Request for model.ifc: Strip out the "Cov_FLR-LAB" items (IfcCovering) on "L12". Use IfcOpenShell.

First a look at what the model holds.

```python
import ifcopenshell
import ifcopenshell.util.element

model = ifcopenshell.open("model.ifc")
print(model.schema)
storey = next(s for s in model.by_type("IfcBuildingStorey") if s.Name == "L12")
coverings = [e for e in ifcopenshell.util.element.get_decomposition(storey) if e.is_a("IfcCovering")]
seen = {}
for e in coverings:
    element_type = ifcopenshell.util.element.get_type(e)
    name = element_type.Name if element_type not in (None, e) else None
    seen[name] = seen.get(name, 0) + 1
for name, count in sorted(seen.items(), key=str):
    print(count, "x", name)
```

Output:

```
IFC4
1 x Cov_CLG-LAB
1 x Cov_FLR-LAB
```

```python
import ifcopenshell
import ifcopenshell.api.root
import ifcopenshell.util.element

model = ifcopenshell.open("model.ifc")

storey = next(s for s in model.by_type("IfcBuildingStorey") if s.Name == "L12")
coverings = [e for e in ifcopenshell.util.element.get_decomposition(storey) if e.is_a("IfcCovering")]
targets = [e for e in coverings if (t := ifcopenshell.util.element.get_type(e)) not in (None, e) and t.Name == "Cov_FLR-LAB"]

for e in targets:
    ifcopenshell.api.root.remove_product(model, product=e)
print(len(targets), "removed")

model.write("model-out.ifc")
```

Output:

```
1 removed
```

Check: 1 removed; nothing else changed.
